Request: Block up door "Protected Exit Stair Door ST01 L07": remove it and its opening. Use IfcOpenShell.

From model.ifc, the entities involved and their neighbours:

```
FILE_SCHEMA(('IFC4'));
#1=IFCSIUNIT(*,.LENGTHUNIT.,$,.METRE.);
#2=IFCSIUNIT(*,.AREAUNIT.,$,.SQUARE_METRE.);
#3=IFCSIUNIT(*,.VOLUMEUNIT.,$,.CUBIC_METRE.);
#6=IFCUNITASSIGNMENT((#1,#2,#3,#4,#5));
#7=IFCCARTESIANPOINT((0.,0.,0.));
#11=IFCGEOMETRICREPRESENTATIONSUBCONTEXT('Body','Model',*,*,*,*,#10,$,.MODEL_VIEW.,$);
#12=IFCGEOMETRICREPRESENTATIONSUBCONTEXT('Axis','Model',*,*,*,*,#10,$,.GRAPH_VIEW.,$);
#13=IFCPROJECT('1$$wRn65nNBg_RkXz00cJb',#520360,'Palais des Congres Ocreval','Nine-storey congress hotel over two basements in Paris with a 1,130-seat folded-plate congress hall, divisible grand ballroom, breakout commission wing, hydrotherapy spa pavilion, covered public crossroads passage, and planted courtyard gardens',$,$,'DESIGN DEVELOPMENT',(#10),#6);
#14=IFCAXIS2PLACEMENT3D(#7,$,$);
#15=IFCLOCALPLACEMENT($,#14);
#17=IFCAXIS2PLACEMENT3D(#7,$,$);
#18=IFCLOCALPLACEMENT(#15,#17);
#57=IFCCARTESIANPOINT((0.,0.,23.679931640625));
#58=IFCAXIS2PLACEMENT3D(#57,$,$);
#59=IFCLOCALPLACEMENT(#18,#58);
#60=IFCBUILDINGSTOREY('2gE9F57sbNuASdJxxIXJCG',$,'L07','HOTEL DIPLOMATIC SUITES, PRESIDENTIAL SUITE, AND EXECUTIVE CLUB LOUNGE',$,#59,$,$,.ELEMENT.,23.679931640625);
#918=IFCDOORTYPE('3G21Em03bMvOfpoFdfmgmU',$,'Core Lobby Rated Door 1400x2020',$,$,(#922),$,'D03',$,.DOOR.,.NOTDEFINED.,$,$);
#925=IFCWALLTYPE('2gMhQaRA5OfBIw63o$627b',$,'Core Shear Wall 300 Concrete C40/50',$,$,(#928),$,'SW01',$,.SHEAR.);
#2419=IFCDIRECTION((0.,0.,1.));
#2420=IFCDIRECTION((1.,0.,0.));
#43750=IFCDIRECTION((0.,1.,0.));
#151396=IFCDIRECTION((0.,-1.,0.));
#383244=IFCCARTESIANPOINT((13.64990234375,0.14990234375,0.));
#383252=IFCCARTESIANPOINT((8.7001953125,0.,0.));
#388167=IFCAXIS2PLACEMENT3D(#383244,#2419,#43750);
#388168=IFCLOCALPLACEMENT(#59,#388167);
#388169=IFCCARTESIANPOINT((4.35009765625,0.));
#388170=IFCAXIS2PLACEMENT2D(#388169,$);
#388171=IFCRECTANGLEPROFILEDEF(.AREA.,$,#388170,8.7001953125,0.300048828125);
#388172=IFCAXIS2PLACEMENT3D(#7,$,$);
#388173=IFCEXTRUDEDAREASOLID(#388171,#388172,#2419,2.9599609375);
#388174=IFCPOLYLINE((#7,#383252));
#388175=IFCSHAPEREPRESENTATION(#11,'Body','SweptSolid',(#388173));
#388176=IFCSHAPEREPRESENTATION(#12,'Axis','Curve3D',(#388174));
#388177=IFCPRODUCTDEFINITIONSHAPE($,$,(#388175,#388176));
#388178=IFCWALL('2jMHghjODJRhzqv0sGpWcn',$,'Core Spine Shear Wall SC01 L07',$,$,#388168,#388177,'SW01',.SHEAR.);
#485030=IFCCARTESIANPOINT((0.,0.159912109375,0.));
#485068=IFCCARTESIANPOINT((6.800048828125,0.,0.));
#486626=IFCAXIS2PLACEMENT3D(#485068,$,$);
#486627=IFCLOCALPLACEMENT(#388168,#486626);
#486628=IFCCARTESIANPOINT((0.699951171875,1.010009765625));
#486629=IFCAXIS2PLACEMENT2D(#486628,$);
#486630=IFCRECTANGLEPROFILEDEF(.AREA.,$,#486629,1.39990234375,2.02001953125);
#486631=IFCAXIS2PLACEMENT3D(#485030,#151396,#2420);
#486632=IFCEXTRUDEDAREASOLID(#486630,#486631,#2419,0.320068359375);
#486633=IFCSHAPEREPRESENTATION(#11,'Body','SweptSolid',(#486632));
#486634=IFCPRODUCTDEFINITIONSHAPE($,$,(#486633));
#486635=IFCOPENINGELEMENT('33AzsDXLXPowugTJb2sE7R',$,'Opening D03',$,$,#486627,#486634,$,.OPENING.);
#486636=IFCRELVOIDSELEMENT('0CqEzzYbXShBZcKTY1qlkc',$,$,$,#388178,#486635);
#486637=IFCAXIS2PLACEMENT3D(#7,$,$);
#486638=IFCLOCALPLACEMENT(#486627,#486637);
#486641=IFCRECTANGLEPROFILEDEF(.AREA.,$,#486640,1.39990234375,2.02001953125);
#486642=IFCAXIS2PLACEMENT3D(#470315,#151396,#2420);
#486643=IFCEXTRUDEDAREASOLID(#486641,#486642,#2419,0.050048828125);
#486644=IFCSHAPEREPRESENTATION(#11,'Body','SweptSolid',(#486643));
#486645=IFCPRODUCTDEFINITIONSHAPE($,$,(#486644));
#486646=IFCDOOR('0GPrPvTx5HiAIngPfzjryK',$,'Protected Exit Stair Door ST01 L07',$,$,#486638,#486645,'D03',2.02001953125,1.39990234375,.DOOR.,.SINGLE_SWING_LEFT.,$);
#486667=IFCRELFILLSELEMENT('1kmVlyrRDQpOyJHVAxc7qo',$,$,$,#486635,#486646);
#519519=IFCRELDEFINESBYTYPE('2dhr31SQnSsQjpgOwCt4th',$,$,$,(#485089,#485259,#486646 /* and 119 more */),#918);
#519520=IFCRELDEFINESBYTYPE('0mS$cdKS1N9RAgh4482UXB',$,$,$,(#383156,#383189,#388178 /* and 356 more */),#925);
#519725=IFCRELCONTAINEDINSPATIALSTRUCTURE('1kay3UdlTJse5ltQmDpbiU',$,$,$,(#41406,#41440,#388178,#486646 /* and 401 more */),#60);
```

```python
import ifcopenshell
import ifcopenshell.api.feature
import ifcopenshell.api.root
import ifcopenshell.geom
import ifcopenshell.util.shape

model = ifcopenshell.open("model.ifc")
settings = ifcopenshell.geom.settings()


def volume(element):
    """Net volume in cubic metres, openings subtracted."""
    shape = ifcopenshell.geom.create_shape(settings, element)
    return ifcopenshell.util.shape.get_volume(shape.geometry)


door = model.by_guid("0GPrPvTx5HiAIngPfzjryK")
opening = door.FillsVoids[0].RelatingOpeningElement
wall = opening.VoidsElements[0].RelatingBuildingElement
before = volume(wall)

ifcopenshell.api.root.remove_product(model, product=door)
ifcopenshell.api.feature.remove_feature(model, feature=opening)

after = volume(wall)

print(f"wall volume {before:.3f} -> {after:.3f} m3")

model.write("model_edited.ifc")
```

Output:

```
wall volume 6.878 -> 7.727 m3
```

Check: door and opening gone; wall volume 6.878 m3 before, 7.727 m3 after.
